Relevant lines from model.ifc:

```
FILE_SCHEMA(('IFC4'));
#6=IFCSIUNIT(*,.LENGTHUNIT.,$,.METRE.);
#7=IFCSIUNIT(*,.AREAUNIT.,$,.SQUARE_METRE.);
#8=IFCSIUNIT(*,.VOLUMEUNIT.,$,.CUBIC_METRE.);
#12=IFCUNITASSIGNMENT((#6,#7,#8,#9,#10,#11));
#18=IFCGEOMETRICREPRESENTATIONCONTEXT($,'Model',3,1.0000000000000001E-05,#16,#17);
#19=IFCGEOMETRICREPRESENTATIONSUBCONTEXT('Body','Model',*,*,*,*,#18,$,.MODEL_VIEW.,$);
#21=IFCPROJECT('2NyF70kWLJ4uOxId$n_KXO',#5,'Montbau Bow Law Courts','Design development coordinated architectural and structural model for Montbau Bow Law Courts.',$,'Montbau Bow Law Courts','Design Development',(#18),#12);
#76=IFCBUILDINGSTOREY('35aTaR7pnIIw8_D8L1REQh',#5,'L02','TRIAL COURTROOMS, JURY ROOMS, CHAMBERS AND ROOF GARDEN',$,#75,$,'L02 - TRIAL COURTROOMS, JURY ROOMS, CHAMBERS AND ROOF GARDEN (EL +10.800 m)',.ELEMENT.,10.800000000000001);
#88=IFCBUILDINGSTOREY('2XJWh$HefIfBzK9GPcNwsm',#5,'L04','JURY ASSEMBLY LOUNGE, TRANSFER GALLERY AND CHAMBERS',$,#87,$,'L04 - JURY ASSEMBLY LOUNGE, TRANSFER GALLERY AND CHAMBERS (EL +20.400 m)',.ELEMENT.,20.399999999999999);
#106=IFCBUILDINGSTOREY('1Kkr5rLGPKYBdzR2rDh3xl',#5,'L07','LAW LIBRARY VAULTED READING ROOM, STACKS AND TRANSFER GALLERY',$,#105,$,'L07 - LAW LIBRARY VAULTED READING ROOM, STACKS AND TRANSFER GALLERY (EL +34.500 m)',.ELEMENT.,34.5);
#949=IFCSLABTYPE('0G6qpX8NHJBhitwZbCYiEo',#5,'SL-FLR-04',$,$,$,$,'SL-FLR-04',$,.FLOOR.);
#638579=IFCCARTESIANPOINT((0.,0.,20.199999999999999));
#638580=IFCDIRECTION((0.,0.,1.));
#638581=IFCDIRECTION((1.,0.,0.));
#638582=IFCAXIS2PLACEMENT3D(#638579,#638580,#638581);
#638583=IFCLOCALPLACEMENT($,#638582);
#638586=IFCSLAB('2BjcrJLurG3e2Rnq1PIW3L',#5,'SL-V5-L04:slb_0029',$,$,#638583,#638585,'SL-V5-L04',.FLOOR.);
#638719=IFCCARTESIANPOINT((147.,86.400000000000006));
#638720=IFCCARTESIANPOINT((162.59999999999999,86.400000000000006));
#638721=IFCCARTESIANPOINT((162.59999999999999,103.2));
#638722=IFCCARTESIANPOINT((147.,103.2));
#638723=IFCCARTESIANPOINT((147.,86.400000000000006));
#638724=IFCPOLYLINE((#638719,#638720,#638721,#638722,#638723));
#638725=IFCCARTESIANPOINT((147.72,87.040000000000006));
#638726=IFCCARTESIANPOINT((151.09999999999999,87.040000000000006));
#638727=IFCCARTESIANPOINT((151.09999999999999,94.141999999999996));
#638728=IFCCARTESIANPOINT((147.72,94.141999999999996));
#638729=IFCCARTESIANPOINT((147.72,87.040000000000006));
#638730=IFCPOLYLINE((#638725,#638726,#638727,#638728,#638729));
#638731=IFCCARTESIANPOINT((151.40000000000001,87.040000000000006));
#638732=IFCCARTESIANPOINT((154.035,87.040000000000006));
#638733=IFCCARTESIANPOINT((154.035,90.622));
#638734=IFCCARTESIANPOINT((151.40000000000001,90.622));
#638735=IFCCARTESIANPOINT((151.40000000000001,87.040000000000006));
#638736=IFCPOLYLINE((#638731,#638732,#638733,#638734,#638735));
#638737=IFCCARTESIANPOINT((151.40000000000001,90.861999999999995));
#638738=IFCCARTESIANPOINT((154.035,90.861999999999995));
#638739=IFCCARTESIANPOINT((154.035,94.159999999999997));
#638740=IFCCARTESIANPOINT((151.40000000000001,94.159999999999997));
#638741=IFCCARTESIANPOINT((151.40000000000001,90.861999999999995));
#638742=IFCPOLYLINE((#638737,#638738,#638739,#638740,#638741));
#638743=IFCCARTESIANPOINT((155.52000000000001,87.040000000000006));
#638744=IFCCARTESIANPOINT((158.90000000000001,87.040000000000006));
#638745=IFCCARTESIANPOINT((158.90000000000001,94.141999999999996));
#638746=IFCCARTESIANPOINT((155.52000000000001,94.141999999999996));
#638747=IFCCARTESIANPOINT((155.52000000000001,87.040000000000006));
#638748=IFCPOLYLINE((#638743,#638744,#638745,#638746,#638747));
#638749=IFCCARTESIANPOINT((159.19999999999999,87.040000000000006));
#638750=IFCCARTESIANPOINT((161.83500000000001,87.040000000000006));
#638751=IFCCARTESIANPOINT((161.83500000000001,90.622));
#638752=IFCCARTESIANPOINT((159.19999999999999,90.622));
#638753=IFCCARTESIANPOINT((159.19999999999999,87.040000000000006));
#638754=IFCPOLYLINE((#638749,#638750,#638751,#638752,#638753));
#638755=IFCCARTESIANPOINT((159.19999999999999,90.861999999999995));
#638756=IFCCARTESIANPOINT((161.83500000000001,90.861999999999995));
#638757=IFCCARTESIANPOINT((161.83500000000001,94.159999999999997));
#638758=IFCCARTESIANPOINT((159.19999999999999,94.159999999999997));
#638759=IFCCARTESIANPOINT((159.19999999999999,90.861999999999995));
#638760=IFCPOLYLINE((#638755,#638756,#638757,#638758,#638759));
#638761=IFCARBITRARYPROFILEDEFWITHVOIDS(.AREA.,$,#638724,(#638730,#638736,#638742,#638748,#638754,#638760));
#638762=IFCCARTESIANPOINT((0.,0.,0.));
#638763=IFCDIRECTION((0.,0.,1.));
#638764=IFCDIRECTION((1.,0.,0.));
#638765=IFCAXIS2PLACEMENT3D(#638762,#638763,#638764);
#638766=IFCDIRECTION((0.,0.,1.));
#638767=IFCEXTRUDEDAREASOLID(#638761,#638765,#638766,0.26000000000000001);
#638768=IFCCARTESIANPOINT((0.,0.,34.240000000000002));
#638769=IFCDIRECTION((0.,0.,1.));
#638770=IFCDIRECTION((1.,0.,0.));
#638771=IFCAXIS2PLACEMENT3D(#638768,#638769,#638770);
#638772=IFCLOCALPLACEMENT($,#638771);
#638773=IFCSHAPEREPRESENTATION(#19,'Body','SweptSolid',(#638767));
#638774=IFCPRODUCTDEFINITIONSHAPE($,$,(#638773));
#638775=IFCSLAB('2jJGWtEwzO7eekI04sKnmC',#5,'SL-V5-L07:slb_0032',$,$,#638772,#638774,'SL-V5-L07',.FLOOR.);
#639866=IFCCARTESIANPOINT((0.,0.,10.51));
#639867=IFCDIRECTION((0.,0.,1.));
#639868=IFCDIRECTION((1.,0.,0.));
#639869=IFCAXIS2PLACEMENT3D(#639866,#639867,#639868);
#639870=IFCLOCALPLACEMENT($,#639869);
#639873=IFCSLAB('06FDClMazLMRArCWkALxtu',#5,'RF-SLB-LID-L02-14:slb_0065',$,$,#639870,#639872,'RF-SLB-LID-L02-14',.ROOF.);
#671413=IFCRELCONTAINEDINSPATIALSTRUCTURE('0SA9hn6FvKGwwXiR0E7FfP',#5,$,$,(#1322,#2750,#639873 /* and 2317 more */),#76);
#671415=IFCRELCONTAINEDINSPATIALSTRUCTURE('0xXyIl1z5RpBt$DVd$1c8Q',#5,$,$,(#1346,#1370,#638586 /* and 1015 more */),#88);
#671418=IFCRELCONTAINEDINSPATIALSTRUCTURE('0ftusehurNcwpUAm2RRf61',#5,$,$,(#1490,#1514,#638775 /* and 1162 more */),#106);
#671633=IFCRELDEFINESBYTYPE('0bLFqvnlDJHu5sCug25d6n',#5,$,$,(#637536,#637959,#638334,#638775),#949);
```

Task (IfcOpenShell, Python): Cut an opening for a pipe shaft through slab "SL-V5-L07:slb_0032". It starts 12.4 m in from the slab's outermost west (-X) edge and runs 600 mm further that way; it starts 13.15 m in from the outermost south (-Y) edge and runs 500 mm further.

```python
import numpy as np
import ifcopenshell
import ifcopenshell.api.feature
import ifcopenshell.api.geometry
import ifcopenshell.api.root
import ifcopenshell.geom
import ifcopenshell.util.placement
import ifcopenshell.util.representation
import ifcopenshell.util.shape
import ifcopenshell.util.unit

model = ifcopenshell.open("model.ifc")
unit_scale = ifcopenshell.util.unit.calculate_unit_scale(model)
settings = ifcopenshell.geom.settings()


def volume(element):
    """Net volume in cubic metres, openings subtracted."""
    shape = ifcopenshell.geom.create_shape(settings, element)
    return ifcopenshell.util.shape.get_volume(shape.geometry)


slab = model.by_guid("2jJGWtEwzO7eekI04sKnmC")
before = volume(slab)

# Extent in the slab's own axes, in metres. The edges named are its -X and -Y sides.
slab_shape = ifcopenshell.geom.create_shape(settings, slab)
vertices = ifcopenshell.util.shape.get_vertices(slab_shape.geometry)
x_min, y_min, bottom = vertices.min(axis=0)
top = vertices[:, 2].max()

opening = ifcopenshell.api.root.create_entity(model, ifc_class="IfcOpeningElement", name="Pipe shaft opening", predefined_type="OPENING")
context = ifcopenshell.util.representation.get_context(model, "Model", "Body", "MODEL_VIEW")
width, depth = 0.6, 0.5
outline = [(0.0, 0.0), (width, 0.0), (width, depth), (0.0, depth), (0.0, 0.0)]
# Overshoot both faces by 50 mm so the cut is clean.
shape = ifcopenshell.api.geometry.add_slab_representation(
    model, context=context, depth=top - bottom + 0.1, polyline=outline
)
ifcopenshell.api.geometry.assign_representation(model, product=opening, representation=shape)

matrix = ifcopenshell.util.placement.get_local_placement(slab.ObjectPlacement)
matrix[:, 3] = matrix @ np.append(np.array([x_min + 12.4, y_min + 13.15, bottom - 0.05]) / unit_scale, 1.0)
ifcopenshell.api.geometry.edit_object_placement(model, product=opening, matrix=matrix, is_si=False)
ifcopenshell.api.feature.add_feature(model, feature=opening, element=slab)

after = volume(slab)

print(f"slab volume {before:.3f} -> {after:.3f} m3")

model.write("model_updated.ifc")
```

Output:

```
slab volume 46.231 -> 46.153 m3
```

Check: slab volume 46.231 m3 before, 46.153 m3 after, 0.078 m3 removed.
